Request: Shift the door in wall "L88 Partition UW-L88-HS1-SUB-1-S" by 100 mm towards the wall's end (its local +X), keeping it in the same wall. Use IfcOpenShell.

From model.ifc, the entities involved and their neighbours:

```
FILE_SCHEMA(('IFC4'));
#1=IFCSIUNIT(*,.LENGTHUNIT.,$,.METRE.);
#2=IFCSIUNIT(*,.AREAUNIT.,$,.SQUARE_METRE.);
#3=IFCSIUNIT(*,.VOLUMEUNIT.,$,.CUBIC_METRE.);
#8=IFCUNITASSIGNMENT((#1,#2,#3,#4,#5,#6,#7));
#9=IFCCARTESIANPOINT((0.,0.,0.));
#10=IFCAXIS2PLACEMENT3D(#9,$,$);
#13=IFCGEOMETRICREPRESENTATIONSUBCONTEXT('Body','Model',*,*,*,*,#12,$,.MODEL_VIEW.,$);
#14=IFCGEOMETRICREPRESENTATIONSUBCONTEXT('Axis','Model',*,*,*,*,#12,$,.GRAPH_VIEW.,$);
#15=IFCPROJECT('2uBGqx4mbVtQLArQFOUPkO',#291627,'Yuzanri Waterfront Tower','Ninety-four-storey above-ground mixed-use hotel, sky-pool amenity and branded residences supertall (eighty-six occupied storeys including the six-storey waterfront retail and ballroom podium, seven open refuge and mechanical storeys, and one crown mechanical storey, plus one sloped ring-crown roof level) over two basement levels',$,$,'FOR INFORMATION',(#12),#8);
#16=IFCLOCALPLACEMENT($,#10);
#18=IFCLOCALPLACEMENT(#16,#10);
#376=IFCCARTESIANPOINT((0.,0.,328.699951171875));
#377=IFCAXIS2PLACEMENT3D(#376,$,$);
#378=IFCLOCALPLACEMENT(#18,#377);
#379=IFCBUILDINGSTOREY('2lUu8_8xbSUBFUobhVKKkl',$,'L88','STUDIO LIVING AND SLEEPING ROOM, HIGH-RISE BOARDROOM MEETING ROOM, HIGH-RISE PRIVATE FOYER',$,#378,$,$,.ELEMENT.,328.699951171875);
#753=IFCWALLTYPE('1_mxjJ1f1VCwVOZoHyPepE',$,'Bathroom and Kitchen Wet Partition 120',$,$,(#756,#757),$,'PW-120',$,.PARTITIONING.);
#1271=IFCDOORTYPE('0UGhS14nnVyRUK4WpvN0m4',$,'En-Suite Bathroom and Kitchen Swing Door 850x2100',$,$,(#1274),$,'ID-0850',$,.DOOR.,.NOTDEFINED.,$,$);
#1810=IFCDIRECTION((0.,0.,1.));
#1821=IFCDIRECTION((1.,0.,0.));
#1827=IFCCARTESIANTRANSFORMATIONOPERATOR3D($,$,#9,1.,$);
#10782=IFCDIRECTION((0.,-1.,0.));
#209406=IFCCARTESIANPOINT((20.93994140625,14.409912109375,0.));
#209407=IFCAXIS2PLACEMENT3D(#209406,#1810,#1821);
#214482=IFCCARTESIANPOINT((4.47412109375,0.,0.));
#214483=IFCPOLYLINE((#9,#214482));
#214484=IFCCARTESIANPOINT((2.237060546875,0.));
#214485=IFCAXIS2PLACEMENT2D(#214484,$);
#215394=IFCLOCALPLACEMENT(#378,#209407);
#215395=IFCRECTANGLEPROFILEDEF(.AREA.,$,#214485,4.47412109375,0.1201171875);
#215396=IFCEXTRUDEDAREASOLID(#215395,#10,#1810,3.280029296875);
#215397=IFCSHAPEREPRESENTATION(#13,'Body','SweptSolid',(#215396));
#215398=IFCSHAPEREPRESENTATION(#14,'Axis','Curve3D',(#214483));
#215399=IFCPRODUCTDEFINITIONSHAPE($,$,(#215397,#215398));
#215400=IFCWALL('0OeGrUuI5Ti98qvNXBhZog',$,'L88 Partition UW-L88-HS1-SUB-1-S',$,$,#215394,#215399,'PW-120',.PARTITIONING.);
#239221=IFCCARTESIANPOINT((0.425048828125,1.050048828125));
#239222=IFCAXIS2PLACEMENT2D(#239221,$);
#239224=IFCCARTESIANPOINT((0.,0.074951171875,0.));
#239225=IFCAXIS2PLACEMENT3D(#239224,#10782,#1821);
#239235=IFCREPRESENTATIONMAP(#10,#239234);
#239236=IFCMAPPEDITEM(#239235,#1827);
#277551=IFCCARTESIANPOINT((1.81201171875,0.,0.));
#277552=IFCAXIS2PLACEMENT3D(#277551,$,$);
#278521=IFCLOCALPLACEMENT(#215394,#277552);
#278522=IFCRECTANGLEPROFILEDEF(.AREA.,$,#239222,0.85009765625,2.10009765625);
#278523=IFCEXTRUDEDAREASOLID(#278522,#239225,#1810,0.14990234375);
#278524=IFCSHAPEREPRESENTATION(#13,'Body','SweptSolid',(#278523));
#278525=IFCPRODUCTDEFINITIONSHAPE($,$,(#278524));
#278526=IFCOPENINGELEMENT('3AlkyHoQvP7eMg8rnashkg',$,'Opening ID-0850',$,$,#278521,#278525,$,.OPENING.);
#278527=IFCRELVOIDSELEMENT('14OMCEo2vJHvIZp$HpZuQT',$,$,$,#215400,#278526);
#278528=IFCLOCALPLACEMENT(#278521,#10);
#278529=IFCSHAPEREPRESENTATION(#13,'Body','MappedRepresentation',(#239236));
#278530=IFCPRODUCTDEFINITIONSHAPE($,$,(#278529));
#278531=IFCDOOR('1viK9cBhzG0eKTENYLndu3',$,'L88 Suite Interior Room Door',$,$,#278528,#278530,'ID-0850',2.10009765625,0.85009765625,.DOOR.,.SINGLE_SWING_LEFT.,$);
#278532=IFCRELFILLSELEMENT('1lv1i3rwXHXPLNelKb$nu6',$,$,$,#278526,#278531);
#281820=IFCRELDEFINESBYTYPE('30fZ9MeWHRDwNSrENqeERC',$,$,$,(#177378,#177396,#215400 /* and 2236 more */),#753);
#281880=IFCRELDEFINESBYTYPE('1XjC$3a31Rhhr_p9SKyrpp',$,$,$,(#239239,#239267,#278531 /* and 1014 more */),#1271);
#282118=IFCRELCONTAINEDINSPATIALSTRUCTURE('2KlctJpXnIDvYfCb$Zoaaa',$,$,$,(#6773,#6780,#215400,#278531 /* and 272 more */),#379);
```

```python
import ifcopenshell
import ifcopenshell.api.geometry
import ifcopenshell.util.placement
import ifcopenshell.util.unit

model = ifcopenshell.open("model.ifc")
unit_scale = ifcopenshell.util.unit.calculate_unit_scale(model)

door = model.by_guid("1viK9cBhzG0eKTENYLndu3")
opening = door.FillsVoids[0].RelatingOpeningElement
wall = opening.VoidsElements[0].RelatingBuildingElement

wall_matrix = ifcopenshell.util.placement.get_local_placement(wall.ObjectPlacement)
shift = wall_matrix[:3, 0] * 0.1 / unit_scale
before = ifcopenshell.util.placement.get_local_placement(door.ObjectPlacement)[:3, 3].copy()

# The door is placed relative to its opening, so it follows when the opening moves.
matrix = ifcopenshell.util.placement.get_local_placement(opening.ObjectPlacement)
matrix[:3, 3] += shift
ifcopenshell.api.geometry.edit_object_placement(
    model, product=opening, matrix=matrix, is_si=False, should_transform_children=True
)

after = ifcopenshell.util.placement.get_local_placement(door.ObjectPlacement)[:3, 3]
print("door moved by", (after - before).round(3) + 0.0)

model.write("model-out.ifc")
```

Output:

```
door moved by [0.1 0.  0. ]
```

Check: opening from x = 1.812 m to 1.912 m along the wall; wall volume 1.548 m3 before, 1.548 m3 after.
